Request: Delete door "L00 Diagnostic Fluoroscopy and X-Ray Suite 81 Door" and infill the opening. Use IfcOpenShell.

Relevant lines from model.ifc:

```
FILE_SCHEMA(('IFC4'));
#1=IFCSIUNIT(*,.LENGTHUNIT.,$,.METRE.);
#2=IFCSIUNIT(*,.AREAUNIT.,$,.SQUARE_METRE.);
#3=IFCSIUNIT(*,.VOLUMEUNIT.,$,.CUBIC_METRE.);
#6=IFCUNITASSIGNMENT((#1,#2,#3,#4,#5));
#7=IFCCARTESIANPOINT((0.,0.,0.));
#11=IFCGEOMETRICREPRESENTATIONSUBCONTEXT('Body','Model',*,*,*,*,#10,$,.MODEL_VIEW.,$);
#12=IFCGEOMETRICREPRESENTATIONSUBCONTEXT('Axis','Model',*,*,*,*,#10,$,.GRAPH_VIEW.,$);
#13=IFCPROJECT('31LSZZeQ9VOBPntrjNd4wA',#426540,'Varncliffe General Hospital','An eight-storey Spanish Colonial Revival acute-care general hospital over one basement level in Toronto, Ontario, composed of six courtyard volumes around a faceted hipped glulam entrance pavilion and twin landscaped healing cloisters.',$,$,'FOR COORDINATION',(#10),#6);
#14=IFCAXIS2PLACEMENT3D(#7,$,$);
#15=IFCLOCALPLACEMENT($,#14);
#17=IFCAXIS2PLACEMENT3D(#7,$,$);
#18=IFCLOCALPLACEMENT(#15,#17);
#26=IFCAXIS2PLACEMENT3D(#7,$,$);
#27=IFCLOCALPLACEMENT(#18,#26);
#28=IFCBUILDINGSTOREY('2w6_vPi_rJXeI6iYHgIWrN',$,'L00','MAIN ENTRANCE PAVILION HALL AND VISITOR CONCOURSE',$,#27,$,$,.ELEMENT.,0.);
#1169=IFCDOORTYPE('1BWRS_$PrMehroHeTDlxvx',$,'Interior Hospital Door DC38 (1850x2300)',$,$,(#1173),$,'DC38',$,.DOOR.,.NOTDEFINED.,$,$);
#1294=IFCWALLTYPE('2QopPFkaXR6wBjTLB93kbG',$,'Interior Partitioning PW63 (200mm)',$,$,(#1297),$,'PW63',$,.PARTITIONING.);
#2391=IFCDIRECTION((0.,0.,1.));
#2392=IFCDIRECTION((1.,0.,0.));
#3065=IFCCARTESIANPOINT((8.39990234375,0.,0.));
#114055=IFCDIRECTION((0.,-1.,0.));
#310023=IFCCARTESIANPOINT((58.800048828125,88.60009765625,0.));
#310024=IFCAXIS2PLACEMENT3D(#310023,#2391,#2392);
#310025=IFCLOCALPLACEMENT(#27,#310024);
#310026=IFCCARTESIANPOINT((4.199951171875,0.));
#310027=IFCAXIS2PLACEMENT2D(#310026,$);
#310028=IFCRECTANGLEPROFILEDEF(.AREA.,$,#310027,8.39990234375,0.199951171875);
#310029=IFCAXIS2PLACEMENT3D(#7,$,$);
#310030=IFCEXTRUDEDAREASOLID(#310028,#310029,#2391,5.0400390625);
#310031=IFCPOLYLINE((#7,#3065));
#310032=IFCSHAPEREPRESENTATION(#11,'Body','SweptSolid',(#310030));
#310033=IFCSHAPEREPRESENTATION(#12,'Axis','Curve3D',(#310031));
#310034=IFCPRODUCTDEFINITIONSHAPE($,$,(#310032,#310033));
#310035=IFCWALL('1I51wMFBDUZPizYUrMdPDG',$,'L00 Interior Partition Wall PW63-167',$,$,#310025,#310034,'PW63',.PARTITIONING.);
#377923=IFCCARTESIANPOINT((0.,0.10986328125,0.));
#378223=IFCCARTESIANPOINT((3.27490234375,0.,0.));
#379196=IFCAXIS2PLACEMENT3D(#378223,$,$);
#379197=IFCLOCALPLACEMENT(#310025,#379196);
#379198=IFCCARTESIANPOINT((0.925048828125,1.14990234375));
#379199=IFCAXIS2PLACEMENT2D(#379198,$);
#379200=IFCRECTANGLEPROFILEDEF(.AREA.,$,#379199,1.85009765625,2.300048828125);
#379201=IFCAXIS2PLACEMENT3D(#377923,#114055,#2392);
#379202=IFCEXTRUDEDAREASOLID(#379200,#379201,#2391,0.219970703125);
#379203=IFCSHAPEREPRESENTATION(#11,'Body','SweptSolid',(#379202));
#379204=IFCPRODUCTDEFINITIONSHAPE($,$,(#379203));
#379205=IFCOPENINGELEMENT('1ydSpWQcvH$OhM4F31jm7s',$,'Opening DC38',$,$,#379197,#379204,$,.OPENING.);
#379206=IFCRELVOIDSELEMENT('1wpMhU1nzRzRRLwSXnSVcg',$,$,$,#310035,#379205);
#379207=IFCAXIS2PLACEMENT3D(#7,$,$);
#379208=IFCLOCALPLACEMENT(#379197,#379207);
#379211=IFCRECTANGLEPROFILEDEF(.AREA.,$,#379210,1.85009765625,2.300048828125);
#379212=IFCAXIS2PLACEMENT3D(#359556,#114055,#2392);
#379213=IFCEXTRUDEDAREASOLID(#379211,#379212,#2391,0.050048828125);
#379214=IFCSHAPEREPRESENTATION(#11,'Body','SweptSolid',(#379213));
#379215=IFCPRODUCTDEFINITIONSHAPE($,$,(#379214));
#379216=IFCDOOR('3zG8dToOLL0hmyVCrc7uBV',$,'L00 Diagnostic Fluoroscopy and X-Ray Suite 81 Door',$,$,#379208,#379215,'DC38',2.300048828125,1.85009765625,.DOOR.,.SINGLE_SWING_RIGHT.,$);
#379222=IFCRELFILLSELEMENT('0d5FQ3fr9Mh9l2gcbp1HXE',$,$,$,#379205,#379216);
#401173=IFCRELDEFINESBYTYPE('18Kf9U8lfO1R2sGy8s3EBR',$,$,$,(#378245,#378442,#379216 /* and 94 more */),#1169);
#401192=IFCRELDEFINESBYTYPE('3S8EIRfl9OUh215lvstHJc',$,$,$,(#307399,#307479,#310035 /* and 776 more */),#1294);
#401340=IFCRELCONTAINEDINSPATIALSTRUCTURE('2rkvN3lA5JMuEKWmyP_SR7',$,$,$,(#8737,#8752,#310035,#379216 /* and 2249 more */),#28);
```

```python
import ifcopenshell
import ifcopenshell.api.feature
import ifcopenshell.api.root
import ifcopenshell.geom
import ifcopenshell.util.shape

model = ifcopenshell.open("model.ifc")
settings = ifcopenshell.geom.settings()


def volume(element):
    """Net volume in cubic metres, openings subtracted."""
    shape = ifcopenshell.geom.create_shape(settings, element)
    return ifcopenshell.util.shape.get_volume(shape.geometry)


door = model.by_guid("3zG8dToOLL0hmyVCrc7uBV")
opening = door.FillsVoids[0].RelatingOpeningElement
wall = opening.VoidsElements[0].RelatingBuildingElement
before = volume(wall)

ifcopenshell.api.root.remove_product(model, product=door)
ifcopenshell.api.feature.remove_feature(model, feature=opening)

after = volume(wall)

print(f"wall volume {before:.3f} -> {after:.3f} m3")

model.write("model_rev.ifc")
```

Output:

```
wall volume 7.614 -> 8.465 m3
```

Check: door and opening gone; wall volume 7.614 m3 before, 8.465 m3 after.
